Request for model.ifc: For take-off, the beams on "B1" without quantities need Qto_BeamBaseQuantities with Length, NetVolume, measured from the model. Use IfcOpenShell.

First a look at what the model holds.

```python
import ifcopenshell
import ifcopenshell.util.element
import ifcopenshell.util.unit

model = ifcopenshell.open("model.ifc")
print(model.schema)
for unit_type in ("LENGTHUNIT", "AREAUNIT", "VOLUMEUNIT"):
    print(unit_type, ifcopenshell.util.unit.calculate_unit_scale(model, unit_type))
storey = next(s for s in model.by_type("IfcBuildingStorey") if s.Name == "B1")
beams = [e for e in ifcopenshell.util.element.get_decomposition(storey) if e.is_a("IfcBeam")]
for e in sorted(beams, key=lambda e: e.id()):
    print(e.id(), e.is_a(), e.Name, list(ifcopenshell.util.element.get_psets(e, qtos_only=True)), sep=" | ")
```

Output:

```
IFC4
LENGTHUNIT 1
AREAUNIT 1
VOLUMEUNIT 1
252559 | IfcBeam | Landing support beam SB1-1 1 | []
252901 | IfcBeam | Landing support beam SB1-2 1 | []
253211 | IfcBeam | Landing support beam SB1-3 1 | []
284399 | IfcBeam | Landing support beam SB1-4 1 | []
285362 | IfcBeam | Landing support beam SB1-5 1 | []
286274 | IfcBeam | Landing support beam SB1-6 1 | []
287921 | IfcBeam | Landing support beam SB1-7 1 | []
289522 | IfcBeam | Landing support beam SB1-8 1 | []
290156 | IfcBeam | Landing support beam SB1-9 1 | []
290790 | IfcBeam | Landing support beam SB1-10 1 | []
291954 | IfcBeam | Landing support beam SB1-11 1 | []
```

```python
import ifcopenshell
import ifcopenshell.api.pset
import ifcopenshell.geom
import ifcopenshell.util.element
import ifcopenshell.util.shape
import ifcopenshell.util.unit

model = ifcopenshell.open("model.ifc")
unit_scale = ifcopenshell.util.unit.calculate_unit_scale(model)
volume_scale = ifcopenshell.util.unit.calculate_unit_scale(model, "VOLUMEUNIT")
settings = ifcopenshell.geom.settings()

storey = next(s for s in model.by_type("IfcBuildingStorey") if s.Name == "B1")
beams = [e for e in ifcopenshell.util.element.get_decomposition(storey) if e.is_a("IfcBeam")]

for e in sorted(beams, key=lambda e: e.id()):
    if ifcopenshell.util.element.get_psets(e, qtos_only=True, should_inherit=False):
        continue
    # Geometry comes back in metres, in the element's own axes.
    shape = ifcopenshell.geom.create_shape(settings, e)
    values = {
        "Length": ifcopenshell.util.shape.get_max_xyz(shape.geometry) / unit_scale,
        "NetVolume": ifcopenshell.util.shape.get_volume(shape.geometry) / volume_scale,
    }
    qto = ifcopenshell.api.pset.add_qto(model, product=e, name="Qto_BeamBaseQuantities")
    ifcopenshell.api.pset.edit_qto(model, qto=qto, properties=values)
    print(e.id(), {k: round(v, 3) for k, v in values.items()})

model.write("model-out.ifc")
```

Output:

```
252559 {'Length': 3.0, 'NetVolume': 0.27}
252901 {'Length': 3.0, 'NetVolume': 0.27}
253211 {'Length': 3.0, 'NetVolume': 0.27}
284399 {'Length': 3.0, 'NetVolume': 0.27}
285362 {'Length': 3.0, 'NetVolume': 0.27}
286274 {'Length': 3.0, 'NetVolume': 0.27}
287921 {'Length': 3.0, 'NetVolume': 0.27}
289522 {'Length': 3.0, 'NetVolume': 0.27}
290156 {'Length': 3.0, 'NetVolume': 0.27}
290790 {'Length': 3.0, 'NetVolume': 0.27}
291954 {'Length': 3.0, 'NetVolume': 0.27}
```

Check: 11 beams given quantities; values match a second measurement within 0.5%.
